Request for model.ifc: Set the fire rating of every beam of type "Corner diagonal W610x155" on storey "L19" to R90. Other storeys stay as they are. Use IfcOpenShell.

First a look at what the model holds.

```python
import ifcopenshell
import ifcopenshell.util.element

model = ifcopenshell.open("model.ifc")
print(model.schema)
storey = next(s for s in model.by_type("IfcBuildingStorey") if s.Name == "L19")
beams = [e for e in ifcopenshell.util.element.get_decomposition(storey) if e.is_a("IfcBeam")]
seen = {}
for e in beams:
    element_type = ifcopenshell.util.element.get_type(e)
    key = (element_type.Name if element_type != e and element_type else None, ifcopenshell.util.element.get_pset(e, "Pset_BeamCommon", "FireRating"))
    seen[key] = seen.get(key, 0) + 1
for (name, value), count in sorted(seen.items(), key=str):
    print(count, "x", name, "|", value)
```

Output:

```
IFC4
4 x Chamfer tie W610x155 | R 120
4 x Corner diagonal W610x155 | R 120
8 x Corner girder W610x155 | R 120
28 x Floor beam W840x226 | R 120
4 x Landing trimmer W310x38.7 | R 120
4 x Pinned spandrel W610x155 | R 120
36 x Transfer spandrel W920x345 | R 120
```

```python
import ifcopenshell
import ifcopenshell.api.pset
import ifcopenshell.util.element

model = ifcopenshell.open("model.ifc")

storey = next(s for s in model.by_type("IfcBuildingStorey") if s.Name == "L19")
beams = [e for e in ifcopenshell.util.element.get_decomposition(storey) if e.is_a("IfcBeam")]

count = 0
for e in beams:
    element_type = ifcopenshell.util.element.get_type(e)
    if element_type in (None, e) or element_type.Name != "Corner diagonal W610x155":
        continue
    found = ifcopenshell.util.element.get_pset(e, "Pset_BeamCommon", should_inherit=False)
    if found:
        pset = model.by_id(found["id"])
        if len(ifcopenshell.util.element.get_elements_by_pset(pset)) > 1:
            pset = ifcopenshell.api.pset.unshare_pset(model, products=[e], pset=pset)[0]
    else:
        pset = ifcopenshell.api.pset.add_pset(model, product=e, name="Pset_BeamCommon")
    ifcopenshell.api.pset.edit_pset(model, pset=pset, properties={"FireRating": "R90"})
    count += 1

print(count, "beams updated")

model.write("model_v2.ifc")
```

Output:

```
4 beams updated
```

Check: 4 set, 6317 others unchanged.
